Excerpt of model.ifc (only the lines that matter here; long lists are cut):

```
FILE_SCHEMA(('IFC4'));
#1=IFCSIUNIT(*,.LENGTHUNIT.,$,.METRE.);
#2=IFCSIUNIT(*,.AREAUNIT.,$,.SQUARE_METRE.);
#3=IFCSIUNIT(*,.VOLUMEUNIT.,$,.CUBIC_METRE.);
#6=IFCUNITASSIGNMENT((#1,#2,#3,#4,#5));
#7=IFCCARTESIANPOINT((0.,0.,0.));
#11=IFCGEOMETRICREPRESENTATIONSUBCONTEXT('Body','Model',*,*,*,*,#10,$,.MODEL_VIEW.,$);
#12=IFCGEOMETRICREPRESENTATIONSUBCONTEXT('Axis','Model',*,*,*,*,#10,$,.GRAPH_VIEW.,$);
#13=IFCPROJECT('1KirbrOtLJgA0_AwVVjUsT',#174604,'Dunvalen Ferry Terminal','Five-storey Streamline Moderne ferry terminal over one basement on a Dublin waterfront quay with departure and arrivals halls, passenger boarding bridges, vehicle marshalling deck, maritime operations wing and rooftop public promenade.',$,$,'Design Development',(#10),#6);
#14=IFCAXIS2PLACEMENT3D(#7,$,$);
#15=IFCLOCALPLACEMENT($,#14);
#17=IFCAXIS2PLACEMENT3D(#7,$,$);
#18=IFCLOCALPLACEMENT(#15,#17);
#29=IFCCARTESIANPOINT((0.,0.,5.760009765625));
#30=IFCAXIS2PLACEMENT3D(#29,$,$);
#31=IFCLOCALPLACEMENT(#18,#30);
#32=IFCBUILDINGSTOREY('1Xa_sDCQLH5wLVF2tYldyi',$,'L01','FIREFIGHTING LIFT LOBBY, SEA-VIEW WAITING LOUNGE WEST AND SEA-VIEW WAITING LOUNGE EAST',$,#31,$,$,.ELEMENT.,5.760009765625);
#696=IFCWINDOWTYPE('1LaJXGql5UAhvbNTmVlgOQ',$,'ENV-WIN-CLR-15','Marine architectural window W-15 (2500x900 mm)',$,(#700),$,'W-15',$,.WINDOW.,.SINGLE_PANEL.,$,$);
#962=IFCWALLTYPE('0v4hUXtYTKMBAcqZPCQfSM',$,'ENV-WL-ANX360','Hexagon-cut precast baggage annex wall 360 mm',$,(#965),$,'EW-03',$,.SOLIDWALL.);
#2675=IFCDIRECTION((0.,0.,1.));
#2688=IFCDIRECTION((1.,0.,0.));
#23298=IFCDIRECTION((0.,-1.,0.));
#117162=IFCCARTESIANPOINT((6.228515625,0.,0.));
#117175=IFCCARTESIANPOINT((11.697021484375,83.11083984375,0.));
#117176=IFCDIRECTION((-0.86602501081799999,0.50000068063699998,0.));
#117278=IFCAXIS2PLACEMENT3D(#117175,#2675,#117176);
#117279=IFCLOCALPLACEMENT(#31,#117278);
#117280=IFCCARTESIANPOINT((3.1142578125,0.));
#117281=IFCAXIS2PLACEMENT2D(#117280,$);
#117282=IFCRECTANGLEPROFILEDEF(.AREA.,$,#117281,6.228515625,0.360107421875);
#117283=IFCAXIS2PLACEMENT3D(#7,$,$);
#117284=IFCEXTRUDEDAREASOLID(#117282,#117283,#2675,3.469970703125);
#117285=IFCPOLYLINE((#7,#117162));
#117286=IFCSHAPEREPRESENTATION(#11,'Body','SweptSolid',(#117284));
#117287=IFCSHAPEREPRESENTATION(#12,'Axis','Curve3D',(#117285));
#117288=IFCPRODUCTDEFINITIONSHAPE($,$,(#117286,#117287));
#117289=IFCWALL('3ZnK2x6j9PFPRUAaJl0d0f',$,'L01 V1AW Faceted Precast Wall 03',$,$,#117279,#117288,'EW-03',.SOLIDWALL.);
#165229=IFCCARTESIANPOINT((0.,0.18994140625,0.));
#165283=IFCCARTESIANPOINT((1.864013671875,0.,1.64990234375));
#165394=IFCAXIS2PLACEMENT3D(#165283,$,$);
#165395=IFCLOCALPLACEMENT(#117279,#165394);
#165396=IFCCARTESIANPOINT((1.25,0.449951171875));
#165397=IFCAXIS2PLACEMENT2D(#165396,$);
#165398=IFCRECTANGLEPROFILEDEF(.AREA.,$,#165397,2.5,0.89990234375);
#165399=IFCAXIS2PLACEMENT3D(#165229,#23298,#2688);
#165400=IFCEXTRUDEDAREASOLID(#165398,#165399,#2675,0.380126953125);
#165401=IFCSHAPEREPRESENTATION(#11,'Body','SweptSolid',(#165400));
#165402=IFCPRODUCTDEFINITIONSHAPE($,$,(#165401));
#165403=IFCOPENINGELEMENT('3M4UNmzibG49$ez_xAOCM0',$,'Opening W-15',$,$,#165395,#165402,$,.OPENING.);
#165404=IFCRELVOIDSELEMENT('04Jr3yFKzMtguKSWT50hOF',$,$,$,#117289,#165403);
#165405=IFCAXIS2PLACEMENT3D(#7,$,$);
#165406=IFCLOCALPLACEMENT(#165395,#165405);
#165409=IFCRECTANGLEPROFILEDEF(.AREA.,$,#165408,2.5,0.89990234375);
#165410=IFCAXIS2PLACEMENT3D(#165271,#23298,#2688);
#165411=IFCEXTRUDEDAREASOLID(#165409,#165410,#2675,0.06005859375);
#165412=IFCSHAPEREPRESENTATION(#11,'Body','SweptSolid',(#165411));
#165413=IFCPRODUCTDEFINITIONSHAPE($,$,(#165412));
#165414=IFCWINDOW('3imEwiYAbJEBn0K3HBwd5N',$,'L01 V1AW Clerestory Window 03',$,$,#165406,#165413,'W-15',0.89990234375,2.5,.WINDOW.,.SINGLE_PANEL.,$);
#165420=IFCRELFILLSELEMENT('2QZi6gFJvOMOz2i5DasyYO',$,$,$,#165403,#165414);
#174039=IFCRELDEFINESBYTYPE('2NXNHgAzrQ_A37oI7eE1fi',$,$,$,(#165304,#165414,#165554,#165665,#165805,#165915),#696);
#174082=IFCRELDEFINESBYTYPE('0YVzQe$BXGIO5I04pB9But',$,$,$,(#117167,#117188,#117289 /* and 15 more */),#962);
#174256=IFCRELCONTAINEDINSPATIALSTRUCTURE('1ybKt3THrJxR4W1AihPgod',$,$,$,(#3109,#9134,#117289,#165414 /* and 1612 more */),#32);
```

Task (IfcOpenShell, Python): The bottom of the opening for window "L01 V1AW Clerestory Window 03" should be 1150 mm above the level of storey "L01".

```python
import numpy as np
import ifcopenshell
import ifcopenshell.api.geometry
import ifcopenshell.geom
import ifcopenshell.util.element
import ifcopenshell.util.placement
import ifcopenshell.util.shape
import ifcopenshell.util.unit

model = ifcopenshell.open("model.ifc")
unit_scale = ifcopenshell.util.unit.calculate_unit_scale(model)

window = model.by_id(165414)
opening = window.FillsVoids[0].RelatingOpeningElement
storey = ifcopenshell.util.element.get_container(window, ifc_class="IfcBuildingStorey")
level = ifcopenshell.util.placement.get_local_placement(storey.ObjectPlacement)[2, 3]

# The opening's origin need not be at the sill, so measure its lowest point.
shape = ifcopenshell.geom.create_shape(ifcopenshell.geom.settings(), opening)
bottom = ifcopenshell.util.shape.get_shape_bottom_elevation(shape, shape.geometry) / unit_scale
dz = level + 1.15 - bottom

shift = np.array([0.0, 0.0, dz])
# The window is placed relative to its opening, so it follows when the opening moves.
matrix = ifcopenshell.util.placement.get_local_placement(opening.ObjectPlacement)
matrix[:3, 3] += shift
ifcopenshell.api.geometry.edit_object_placement(
    model, product=opening, matrix=matrix, is_si=False, should_transform_children=True
)

print(f"moved by {dz * unit_scale:+.3f} m")

model.write("model-out.ifc")
```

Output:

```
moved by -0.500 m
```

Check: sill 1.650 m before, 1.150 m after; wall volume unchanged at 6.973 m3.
